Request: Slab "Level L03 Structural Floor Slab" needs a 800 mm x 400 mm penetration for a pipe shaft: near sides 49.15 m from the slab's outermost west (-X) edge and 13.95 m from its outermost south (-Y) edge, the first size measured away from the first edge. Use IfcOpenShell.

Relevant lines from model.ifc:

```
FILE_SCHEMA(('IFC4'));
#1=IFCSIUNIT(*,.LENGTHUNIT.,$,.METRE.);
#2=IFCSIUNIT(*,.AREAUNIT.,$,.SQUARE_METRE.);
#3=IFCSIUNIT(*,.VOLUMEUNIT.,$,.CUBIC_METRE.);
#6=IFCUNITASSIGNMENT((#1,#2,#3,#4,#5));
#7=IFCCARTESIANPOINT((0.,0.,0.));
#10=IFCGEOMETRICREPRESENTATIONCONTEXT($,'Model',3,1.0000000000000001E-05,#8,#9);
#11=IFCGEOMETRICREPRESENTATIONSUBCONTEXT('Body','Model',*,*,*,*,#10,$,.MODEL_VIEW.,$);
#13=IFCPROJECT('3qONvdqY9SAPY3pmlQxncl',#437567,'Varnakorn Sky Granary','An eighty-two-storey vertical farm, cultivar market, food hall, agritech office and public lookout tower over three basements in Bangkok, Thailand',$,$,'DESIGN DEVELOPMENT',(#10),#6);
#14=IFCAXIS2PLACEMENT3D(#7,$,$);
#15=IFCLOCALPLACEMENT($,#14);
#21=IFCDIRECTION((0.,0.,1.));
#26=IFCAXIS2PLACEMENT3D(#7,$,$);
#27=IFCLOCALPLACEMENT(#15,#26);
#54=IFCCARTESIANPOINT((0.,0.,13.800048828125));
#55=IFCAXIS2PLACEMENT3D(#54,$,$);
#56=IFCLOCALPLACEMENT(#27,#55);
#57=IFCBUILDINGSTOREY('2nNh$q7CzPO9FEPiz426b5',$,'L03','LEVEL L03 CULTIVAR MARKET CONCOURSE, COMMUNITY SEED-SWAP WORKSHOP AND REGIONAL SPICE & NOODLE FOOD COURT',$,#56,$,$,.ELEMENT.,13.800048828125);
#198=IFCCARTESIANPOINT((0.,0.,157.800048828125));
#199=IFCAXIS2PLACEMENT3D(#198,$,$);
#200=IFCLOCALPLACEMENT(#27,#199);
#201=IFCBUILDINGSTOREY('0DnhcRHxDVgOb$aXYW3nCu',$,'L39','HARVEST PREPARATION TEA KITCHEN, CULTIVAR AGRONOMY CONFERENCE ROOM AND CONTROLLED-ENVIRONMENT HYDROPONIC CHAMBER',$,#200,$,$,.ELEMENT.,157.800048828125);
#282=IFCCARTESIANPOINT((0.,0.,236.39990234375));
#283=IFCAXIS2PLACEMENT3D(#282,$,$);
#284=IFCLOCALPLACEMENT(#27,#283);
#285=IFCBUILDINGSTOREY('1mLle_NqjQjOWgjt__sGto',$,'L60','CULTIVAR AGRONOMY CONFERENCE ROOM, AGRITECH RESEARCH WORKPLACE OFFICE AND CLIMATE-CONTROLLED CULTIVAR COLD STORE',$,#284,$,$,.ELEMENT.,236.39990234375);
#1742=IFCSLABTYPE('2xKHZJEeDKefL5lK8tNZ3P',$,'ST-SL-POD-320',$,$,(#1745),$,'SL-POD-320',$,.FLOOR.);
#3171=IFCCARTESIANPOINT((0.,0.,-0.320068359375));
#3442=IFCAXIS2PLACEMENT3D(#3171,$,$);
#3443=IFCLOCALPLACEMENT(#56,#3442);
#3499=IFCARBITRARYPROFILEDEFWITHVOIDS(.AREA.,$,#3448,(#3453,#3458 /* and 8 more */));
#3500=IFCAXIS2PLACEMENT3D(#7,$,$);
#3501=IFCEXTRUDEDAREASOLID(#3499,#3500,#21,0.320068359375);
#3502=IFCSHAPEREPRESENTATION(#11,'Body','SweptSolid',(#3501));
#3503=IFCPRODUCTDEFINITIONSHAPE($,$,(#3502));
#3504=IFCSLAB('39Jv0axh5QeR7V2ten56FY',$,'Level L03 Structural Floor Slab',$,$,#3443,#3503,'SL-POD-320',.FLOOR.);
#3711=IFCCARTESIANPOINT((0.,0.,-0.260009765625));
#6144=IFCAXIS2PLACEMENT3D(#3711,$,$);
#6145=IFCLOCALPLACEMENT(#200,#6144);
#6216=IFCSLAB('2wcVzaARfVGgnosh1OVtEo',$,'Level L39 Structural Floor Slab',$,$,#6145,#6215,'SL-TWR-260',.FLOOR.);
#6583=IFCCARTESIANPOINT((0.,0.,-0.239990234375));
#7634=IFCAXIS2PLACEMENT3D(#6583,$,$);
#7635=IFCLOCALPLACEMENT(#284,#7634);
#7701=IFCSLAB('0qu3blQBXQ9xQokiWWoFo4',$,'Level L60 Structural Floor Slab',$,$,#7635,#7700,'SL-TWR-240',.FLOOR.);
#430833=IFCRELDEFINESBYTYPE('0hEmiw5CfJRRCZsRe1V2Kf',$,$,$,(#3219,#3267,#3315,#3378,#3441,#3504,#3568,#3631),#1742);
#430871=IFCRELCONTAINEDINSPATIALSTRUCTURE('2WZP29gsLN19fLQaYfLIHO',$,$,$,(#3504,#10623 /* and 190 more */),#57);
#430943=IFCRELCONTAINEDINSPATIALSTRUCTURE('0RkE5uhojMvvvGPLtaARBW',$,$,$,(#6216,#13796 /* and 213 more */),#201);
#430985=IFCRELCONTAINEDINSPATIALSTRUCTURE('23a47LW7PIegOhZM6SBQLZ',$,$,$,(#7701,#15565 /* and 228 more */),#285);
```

```python
import numpy as np
import ifcopenshell
import ifcopenshell.api.feature
import ifcopenshell.api.geometry
import ifcopenshell.api.root
import ifcopenshell.geom
import ifcopenshell.util.placement
import ifcopenshell.util.representation
import ifcopenshell.util.shape
import ifcopenshell.util.unit

model = ifcopenshell.open("model.ifc")
unit_scale = ifcopenshell.util.unit.calculate_unit_scale(model)
settings = ifcopenshell.geom.settings()


def volume(element):
    """Net volume in cubic metres, openings subtracted."""
    shape = ifcopenshell.geom.create_shape(settings, element)
    return ifcopenshell.util.shape.get_volume(shape.geometry)


slab = model.by_guid("39Jv0axh5QeR7V2ten56FY")
before = volume(slab)

# Extent in the slab's own axes, in metres. The edges named are its -X and -Y sides.
slab_shape = ifcopenshell.geom.create_shape(settings, slab)
vertices = ifcopenshell.util.shape.get_vertices(slab_shape.geometry)
x_min, y_min, bottom = vertices.min(axis=0)
top = vertices[:, 2].max()

opening = ifcopenshell.api.root.create_entity(model, ifc_class="IfcOpeningElement", name="Pipe shaft opening", predefined_type="OPENING")
context = ifcopenshell.util.representation.get_context(model, "Model", "Body", "MODEL_VIEW")
width, depth = 0.8, 0.4
outline = [(0.0, 0.0), (width, 0.0), (width, depth), (0.0, depth), (0.0, 0.0)]
# Overshoot both faces by 50 mm so the cut is clean.
shape = ifcopenshell.api.geometry.add_slab_representation(
    model, context=context, depth=top - bottom + 0.1, polyline=outline
)
ifcopenshell.api.geometry.assign_representation(model, product=opening, representation=shape)

matrix = ifcopenshell.util.placement.get_local_placement(slab.ObjectPlacement)
matrix[:, 3] = matrix @ np.append(np.array([x_min + 49.15, y_min + 13.95, bottom - 0.05]) / unit_scale, 1.0)
ifcopenshell.api.geometry.edit_object_placement(model, product=opening, matrix=matrix, is_si=False)
ifcopenshell.api.feature.add_feature(model, feature=opening, element=slab)

after = volume(slab)

print(f"slab volume {before:.3f} -> {after:.3f} m3")

model.write("model_edited.ifc")
```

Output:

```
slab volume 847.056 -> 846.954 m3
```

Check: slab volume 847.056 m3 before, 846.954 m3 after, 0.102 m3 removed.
